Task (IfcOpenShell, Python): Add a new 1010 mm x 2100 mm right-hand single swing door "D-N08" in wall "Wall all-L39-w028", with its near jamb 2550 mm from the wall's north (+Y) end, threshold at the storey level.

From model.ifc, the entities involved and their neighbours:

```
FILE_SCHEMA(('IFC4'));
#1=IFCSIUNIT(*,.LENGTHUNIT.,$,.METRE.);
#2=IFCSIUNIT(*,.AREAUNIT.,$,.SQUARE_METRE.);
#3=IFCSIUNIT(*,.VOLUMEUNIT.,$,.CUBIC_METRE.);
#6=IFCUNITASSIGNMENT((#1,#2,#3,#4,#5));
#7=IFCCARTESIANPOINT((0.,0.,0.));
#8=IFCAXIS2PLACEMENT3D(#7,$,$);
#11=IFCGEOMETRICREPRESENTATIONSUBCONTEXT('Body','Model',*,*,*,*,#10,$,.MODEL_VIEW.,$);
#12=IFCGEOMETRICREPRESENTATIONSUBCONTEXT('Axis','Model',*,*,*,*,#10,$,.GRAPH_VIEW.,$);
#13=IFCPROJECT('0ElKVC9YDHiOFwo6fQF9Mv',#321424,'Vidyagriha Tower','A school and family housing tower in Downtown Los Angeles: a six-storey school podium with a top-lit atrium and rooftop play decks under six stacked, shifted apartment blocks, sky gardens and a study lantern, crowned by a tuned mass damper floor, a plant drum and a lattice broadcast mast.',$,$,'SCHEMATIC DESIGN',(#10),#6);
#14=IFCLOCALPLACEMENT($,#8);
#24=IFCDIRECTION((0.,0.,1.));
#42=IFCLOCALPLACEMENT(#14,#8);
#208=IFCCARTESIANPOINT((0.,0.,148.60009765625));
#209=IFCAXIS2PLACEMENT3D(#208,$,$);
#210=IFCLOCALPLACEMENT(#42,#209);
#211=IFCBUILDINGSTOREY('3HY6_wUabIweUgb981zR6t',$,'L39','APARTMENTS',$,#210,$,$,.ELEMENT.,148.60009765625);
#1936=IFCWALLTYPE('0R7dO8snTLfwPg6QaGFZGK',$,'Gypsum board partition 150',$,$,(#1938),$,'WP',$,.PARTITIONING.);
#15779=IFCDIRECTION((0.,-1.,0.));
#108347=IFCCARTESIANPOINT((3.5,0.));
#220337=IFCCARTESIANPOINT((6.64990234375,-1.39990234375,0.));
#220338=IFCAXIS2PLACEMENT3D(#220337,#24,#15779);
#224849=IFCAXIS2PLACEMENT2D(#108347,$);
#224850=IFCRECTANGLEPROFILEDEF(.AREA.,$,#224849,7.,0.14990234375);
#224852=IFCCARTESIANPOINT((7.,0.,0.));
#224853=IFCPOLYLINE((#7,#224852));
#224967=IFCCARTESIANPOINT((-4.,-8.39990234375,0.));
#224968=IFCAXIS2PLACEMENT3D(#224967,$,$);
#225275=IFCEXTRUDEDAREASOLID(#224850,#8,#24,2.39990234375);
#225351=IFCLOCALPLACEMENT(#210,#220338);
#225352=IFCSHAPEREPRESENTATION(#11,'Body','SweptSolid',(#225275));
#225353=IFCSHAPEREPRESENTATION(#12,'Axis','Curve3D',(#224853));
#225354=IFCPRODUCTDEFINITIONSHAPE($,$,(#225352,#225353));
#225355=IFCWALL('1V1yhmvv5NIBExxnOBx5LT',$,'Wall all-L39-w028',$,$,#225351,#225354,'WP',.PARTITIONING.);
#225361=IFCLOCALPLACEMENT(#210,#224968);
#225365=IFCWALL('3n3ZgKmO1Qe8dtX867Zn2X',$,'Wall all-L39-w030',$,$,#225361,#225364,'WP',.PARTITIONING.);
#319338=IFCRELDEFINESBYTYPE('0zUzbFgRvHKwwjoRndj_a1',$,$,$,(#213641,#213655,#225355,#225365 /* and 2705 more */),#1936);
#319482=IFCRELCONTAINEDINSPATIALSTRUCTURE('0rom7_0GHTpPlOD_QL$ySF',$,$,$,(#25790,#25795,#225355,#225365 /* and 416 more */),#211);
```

```python
import numpy as np
import ifcopenshell
import ifcopenshell.api.feature
import ifcopenshell.api.geometry
import ifcopenshell.api.root
import ifcopenshell.api.spatial
import ifcopenshell.geom
import ifcopenshell.util.element
import ifcopenshell.util.placement
import ifcopenshell.util.representation
import ifcopenshell.util.shape
import ifcopenshell.util.unit

model = ifcopenshell.open("model.ifc")
unit_scale = ifcopenshell.util.unit.calculate_unit_scale(model)
settings = ifcopenshell.geom.settings()


def volume(element):
    """Net volume in cubic metres, openings subtracted."""
    shape = ifcopenshell.geom.create_shape(settings, element)
    return ifcopenshell.util.shape.get_volume(shape.geometry)


wall = model.by_id(225355)
storey = ifcopenshell.util.element.get_container(wall, ifc_class="IfcBuildingStorey")
context = ifcopenshell.util.representation.get_context(model, "Model", "Body", "MODEL_VIEW")
before = volume(wall)

width, height, from_end, sill = 1.01, 2.1, 2.55, 0.0  # metres

# The wall runs along its own X axis, and the end named is its -X end.
wall_shape = ifcopenshell.geom.create_shape(settings, wall)
x, y, z = ifcopenshell.util.shape.get_vertices(wall_shape.geometry).T
start = x.min() + from_end
face, thickness = float(y.min()), float(y.max() - y.min())
wall_matrix = ifcopenshell.util.placement.get_local_placement(wall.ObjectPlacement)
level = ifcopenshell.util.placement.get_local_placement(storey.ObjectPlacement)[2, 3]


def in_wall(x, y):
    """Placement at x, y metres in the wall's axes, at sill height."""
    matrix = wall_matrix.copy()
    matrix[:, 3] = wall_matrix @ np.array([x / unit_scale, y / unit_scale, 0.0, 1.0])
    matrix[2, 3] = level + sill / unit_scale
    return matrix


# Opening: a box that overshoots both wall faces by 50 mm.
opening = ifcopenshell.api.root.create_entity(model, ifc_class="IfcOpeningElement", predefined_type="OPENING")
box = ifcopenshell.api.geometry.add_wall_representation(
    model, context=context, length=width, height=height, thickness=thickness + 0.1
)
ifcopenshell.api.geometry.assign_representation(model, product=opening, representation=box)
ifcopenshell.api.geometry.edit_object_placement(model, product=opening, matrix=in_wall(start, face - 0.05), is_si=False)
ifcopenshell.api.feature.add_feature(model, feature=opening, element=wall)

door = ifcopenshell.api.root.create_entity(model, ifc_class="IfcDoor", name="D-N08", predefined_type="DOOR")
door.OverallWidth, door.OverallHeight = width / unit_scale, height / unit_scale
door.OperationType = "SINGLE_SWING_RIGHT"
body = ifcopenshell.api.geometry.add_door_representation(
    model,
    context=context,
    overall_width=door.OverallWidth,
    overall_height=door.OverallHeight,
    operation_type="SINGLE_SWING_RIGHT",
    lining_properties={"LiningDepth": thickness / unit_scale, "ThresholdDepth": thickness / unit_scale},
)
ifcopenshell.api.geometry.assign_representation(model, product=door, representation=body)
ifcopenshell.api.spatial.assign_container(model, products=[door], relating_structure=storey)
ifcopenshell.api.feature.add_filling(model, opening=opening, element=door)

# The lining spans the wall, so the door starts at the wall face.
ifcopenshell.api.geometry.edit_object_placement(model, product=door, matrix=in_wall(start, face), is_si=False)

after = volume(wall)

print(f"wall volume {before:.3f} -> {after:.3f} m3")

model.write("model_updated.ifc")
```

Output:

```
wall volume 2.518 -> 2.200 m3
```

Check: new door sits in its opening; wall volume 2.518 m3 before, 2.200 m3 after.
